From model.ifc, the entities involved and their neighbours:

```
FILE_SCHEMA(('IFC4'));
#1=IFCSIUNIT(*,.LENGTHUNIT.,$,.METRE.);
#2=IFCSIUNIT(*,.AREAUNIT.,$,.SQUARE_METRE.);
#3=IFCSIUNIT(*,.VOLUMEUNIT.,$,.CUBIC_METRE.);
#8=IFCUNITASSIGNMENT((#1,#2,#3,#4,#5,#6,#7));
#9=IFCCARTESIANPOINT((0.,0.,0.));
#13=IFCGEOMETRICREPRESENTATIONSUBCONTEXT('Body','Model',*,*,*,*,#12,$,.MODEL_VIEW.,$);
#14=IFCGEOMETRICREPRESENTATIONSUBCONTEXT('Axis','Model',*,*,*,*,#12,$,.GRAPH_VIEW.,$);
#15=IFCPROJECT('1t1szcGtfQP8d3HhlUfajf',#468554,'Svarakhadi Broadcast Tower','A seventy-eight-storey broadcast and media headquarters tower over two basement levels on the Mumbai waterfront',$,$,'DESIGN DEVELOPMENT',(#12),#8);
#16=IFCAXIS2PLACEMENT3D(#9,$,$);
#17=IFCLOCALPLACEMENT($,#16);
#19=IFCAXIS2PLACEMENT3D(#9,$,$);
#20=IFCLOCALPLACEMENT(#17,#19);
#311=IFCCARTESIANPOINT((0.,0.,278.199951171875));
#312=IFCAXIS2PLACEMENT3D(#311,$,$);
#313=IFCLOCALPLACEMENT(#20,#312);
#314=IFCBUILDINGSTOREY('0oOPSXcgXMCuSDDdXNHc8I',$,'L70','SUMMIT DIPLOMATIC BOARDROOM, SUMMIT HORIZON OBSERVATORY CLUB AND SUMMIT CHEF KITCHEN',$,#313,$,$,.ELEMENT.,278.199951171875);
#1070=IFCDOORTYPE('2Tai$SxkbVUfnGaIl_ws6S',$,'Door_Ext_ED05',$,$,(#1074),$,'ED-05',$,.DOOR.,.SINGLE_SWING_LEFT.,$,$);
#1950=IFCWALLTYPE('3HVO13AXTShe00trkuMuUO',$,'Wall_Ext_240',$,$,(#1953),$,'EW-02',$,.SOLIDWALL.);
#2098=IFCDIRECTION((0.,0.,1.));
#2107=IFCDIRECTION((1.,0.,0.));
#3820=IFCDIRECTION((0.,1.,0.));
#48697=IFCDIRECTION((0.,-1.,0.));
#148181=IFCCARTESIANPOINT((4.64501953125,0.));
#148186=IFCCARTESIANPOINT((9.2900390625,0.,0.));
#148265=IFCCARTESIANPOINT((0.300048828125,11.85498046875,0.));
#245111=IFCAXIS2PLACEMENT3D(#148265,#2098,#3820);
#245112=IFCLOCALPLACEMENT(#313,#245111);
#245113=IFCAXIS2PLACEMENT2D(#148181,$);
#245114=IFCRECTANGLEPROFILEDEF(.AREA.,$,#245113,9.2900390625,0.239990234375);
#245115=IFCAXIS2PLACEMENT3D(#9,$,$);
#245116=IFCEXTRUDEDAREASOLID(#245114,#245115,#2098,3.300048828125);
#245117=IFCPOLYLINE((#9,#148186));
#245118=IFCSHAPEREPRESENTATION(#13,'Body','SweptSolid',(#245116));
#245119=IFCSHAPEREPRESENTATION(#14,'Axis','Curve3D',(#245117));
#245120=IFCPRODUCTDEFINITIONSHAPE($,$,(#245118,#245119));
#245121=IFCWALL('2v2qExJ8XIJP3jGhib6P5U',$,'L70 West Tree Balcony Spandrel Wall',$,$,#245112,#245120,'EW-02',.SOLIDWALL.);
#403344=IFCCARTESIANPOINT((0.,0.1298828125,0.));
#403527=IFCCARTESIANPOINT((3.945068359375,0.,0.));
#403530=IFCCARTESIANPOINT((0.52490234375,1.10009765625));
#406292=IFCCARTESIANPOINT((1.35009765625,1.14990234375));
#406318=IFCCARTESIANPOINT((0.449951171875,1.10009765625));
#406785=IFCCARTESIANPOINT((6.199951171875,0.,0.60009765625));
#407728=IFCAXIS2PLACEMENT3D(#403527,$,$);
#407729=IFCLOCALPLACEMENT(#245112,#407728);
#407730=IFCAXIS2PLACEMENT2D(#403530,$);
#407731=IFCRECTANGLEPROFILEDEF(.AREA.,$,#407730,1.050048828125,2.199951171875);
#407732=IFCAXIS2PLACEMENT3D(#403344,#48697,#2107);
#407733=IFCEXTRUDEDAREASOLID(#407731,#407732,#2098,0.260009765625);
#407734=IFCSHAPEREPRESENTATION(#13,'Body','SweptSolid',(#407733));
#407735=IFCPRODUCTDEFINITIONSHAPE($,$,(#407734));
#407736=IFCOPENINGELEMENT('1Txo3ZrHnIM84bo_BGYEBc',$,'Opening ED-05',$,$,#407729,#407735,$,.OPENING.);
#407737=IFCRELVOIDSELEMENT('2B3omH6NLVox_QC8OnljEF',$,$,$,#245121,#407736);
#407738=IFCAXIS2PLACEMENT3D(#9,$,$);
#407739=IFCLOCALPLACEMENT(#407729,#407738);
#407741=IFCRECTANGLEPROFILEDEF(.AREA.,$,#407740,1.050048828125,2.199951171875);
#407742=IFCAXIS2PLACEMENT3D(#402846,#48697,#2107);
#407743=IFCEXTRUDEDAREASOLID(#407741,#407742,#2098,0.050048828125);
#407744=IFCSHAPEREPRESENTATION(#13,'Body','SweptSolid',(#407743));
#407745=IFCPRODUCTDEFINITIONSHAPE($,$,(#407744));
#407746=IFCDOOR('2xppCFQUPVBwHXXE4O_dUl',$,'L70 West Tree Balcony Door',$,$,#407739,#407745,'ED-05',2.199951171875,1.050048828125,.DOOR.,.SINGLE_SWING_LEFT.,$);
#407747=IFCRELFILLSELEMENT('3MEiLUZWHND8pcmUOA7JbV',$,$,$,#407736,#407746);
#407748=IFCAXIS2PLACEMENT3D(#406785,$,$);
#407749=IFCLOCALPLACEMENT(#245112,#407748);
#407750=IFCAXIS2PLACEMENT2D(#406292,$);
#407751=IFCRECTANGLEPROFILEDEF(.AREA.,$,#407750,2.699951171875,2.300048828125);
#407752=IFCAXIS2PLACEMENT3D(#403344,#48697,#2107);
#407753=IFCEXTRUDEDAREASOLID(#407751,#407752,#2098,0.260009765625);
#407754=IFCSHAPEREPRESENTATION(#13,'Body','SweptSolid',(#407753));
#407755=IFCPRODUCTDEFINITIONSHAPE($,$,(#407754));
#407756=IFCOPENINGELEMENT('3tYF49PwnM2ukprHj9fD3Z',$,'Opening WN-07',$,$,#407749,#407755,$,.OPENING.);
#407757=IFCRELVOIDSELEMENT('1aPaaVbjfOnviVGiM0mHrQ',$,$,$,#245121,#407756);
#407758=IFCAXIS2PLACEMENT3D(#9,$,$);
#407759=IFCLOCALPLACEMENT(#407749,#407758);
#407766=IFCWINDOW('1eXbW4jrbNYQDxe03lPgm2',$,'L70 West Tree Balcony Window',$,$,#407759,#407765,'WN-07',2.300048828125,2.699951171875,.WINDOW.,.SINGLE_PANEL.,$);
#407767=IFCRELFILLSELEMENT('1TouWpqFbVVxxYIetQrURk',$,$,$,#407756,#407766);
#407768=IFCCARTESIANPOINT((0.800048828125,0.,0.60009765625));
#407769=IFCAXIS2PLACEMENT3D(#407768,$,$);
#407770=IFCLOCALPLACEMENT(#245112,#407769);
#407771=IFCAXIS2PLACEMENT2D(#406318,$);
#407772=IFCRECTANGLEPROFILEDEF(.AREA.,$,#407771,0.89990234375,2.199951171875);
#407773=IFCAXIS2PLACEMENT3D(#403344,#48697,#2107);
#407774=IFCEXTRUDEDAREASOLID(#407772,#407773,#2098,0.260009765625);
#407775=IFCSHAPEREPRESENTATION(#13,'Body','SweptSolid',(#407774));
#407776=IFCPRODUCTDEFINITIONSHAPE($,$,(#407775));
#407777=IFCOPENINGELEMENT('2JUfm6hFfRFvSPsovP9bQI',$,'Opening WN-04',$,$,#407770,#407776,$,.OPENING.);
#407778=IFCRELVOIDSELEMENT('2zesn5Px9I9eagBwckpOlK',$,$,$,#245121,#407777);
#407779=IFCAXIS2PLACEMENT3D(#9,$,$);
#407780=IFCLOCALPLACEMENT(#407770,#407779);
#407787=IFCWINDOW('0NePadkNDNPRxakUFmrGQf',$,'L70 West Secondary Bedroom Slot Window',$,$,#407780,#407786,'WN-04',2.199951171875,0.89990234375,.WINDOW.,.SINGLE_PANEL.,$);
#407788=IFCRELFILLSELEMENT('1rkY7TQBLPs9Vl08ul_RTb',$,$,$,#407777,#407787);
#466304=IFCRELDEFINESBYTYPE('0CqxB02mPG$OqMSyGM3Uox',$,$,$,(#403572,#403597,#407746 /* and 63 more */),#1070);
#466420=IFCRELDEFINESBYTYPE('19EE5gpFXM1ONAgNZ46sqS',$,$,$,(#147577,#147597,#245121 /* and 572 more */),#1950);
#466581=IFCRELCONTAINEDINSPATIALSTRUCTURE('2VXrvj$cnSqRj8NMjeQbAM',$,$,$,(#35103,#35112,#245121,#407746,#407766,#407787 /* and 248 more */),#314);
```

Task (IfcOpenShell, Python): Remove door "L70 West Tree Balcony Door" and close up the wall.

```python
import ifcopenshell
import ifcopenshell.api.feature
import ifcopenshell.api.root
import ifcopenshell.geom
import ifcopenshell.util.shape

model = ifcopenshell.open("model.ifc")
settings = ifcopenshell.geom.settings()


def volume(element):
    """Net volume in cubic metres, openings subtracted."""
    shape = ifcopenshell.geom.create_shape(settings, element)
    return ifcopenshell.util.shape.get_volume(shape.geometry)


door = model.by_guid("2xppCFQUPVBwHXXE4O_dUl")
opening = door.FillsVoids[0].RelatingOpeningElement
wall = opening.VoidsElements[0].RelatingBuildingElement
before = volume(wall)

ifcopenshell.api.root.remove_product(model, product=door)
ifcopenshell.api.feature.remove_feature(model, feature=opening)

after = volume(wall)

print(f"wall volume {before:.3f} -> {after:.3f} m3")

model.write("model-out.ifc")
```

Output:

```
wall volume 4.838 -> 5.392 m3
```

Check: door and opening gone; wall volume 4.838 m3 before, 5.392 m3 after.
